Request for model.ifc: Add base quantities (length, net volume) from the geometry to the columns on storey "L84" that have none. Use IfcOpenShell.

First a look at what the model holds.

```python
import ifcopenshell
import ifcopenshell.util.element
import ifcopenshell.util.unit

model = ifcopenshell.open("model.ifc")
print(model.schema)
for unit_type in ("LENGTHUNIT", "AREAUNIT", "VOLUMEUNIT"):
    print(unit_type, ifcopenshell.util.unit.calculate_unit_scale(model, unit_type))
storey = next(s for s in model.by_type("IfcBuildingStorey") if s.Name == "L84")
columns = [e for e in ifcopenshell.util.element.get_decomposition(storey) if e.is_a("IfcColumn")]
for e in sorted(columns, key=lambda e: e.id()):
    print(e.id(), e.is_a(), e.Name, list(ifcopenshell.util.element.get_psets(e, qtos_only=True)), sep=" | ")
```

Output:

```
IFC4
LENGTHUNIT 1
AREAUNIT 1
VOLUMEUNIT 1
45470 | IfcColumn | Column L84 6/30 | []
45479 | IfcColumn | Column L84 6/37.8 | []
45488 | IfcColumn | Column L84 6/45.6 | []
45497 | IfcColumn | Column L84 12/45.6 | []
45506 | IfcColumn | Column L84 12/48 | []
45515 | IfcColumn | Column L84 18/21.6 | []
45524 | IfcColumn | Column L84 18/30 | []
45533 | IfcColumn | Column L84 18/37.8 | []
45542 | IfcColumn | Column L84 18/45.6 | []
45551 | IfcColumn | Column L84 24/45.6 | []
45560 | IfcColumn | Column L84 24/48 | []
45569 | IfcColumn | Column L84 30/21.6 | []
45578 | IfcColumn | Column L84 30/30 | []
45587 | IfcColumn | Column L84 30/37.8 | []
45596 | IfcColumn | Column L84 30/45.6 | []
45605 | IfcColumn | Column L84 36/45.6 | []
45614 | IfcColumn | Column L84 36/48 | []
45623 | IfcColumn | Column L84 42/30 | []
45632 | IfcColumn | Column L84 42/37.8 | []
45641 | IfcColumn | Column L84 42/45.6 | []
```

```python
import ifcopenshell
import ifcopenshell.api.pset
import ifcopenshell.geom
import ifcopenshell.util.element
import ifcopenshell.util.shape
import ifcopenshell.util.unit

model = ifcopenshell.open("model.ifc")
unit_scale = ifcopenshell.util.unit.calculate_unit_scale(model)
volume_scale = ifcopenshell.util.unit.calculate_unit_scale(model, "VOLUMEUNIT")
settings = ifcopenshell.geom.settings()

storey = next(s for s in model.by_type("IfcBuildingStorey") if s.Name == "L84")
columns = [e for e in ifcopenshell.util.element.get_decomposition(storey) if e.is_a("IfcColumn")]

for e in sorted(columns, key=lambda e: e.id()):
    if ifcopenshell.util.element.get_psets(e, qtos_only=True, should_inherit=False):
        continue
    # Geometry comes back in metres, in the element's own axes.
    shape = ifcopenshell.geom.create_shape(settings, e)
    values = {
        "Length": ifcopenshell.util.shape.get_z(shape.geometry) / unit_scale,
        "NetVolume": ifcopenshell.util.shape.get_volume(shape.geometry) / volume_scale,
    }
    qto = ifcopenshell.api.pset.add_qto(model, product=e, name="Qto_ColumnBaseQuantities")
    ifcopenshell.api.pset.edit_qto(model, qto=qto, properties=values)
    print(e.id(), {k: round(v, 3) for k, v in values.items()})

model.write("model_v2.ifc")
```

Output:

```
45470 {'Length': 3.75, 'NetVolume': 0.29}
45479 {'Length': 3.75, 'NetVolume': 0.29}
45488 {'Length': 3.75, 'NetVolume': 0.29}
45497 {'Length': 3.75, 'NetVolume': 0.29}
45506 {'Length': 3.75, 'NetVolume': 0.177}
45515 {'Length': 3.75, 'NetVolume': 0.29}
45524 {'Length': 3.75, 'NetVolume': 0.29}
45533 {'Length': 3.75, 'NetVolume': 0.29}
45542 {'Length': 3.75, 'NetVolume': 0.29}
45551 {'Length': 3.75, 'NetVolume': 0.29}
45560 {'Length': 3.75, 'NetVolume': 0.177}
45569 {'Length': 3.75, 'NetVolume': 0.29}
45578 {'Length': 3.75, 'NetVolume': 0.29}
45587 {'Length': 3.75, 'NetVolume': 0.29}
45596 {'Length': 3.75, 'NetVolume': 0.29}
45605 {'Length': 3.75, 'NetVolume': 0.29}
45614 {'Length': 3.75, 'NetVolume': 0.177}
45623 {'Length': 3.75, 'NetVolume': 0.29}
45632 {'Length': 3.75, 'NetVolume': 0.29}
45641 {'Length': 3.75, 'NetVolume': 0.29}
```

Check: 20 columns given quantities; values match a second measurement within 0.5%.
